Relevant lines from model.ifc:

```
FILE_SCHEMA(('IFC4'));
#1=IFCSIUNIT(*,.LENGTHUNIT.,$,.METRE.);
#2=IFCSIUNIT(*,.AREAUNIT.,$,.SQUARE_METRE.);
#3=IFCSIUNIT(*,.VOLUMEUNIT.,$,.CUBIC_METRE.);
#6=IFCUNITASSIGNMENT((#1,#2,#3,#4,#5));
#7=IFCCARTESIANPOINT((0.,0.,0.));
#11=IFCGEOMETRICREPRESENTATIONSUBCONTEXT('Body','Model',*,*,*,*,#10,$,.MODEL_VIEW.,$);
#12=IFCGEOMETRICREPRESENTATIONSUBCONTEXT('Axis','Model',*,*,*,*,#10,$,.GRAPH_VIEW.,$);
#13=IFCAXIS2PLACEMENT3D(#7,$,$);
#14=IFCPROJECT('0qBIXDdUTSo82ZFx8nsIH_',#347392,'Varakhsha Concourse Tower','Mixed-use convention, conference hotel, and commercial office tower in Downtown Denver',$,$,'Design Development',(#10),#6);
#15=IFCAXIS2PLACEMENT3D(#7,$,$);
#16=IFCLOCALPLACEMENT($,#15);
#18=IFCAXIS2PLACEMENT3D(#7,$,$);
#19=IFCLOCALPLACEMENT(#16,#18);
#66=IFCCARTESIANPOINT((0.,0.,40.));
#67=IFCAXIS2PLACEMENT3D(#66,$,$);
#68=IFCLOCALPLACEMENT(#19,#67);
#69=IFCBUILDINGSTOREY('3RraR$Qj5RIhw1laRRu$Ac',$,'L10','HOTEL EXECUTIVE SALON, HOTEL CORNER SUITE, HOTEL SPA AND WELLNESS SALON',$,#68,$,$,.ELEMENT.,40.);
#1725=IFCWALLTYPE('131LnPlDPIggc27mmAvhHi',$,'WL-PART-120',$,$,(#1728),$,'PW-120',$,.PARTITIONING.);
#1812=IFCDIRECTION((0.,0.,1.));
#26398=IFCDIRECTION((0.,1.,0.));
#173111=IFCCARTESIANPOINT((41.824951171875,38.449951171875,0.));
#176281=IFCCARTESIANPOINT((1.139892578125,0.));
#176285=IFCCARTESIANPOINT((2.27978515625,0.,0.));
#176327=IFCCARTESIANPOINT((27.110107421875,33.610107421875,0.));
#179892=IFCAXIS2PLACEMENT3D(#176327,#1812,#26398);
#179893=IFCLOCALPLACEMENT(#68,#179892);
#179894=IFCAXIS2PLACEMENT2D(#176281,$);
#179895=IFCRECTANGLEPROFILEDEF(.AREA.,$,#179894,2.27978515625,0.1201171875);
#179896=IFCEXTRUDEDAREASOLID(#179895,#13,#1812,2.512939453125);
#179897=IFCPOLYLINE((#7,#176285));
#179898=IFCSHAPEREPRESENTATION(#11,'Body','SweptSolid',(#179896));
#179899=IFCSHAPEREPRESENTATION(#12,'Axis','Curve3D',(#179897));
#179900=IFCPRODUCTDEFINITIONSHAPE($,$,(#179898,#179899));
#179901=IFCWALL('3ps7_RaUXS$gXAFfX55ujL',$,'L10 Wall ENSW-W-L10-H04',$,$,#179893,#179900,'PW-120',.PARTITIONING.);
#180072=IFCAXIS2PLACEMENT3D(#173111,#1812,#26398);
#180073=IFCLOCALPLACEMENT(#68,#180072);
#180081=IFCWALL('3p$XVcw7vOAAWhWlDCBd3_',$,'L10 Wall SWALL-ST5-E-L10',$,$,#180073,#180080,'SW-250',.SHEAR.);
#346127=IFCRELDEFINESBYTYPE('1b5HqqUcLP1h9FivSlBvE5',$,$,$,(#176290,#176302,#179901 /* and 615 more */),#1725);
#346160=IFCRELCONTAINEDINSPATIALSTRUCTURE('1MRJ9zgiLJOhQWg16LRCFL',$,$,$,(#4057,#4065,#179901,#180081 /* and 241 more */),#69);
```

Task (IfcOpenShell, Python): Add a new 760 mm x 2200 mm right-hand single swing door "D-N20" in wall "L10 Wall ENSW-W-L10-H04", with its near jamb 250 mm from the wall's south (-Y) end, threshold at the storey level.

```python
import numpy as np
import ifcopenshell
import ifcopenshell.api.feature
import ifcopenshell.api.geometry
import ifcopenshell.api.root
import ifcopenshell.api.spatial
import ifcopenshell.geom
import ifcopenshell.util.element
import ifcopenshell.util.placement
import ifcopenshell.util.representation
import ifcopenshell.util.shape
import ifcopenshell.util.unit

model = ifcopenshell.open("model.ifc")
unit_scale = ifcopenshell.util.unit.calculate_unit_scale(model)
settings = ifcopenshell.geom.settings()


def volume(element):
    """Net volume in cubic metres, openings subtracted."""
    shape = ifcopenshell.geom.create_shape(settings, element)
    return ifcopenshell.util.shape.get_volume(shape.geometry)


wall = model.by_guid("3ps7_RaUXS$gXAFfX55ujL")
storey = ifcopenshell.util.element.get_container(wall, ifc_class="IfcBuildingStorey")
context = ifcopenshell.util.representation.get_context(model, "Model", "Body", "MODEL_VIEW")
before = volume(wall)

width, height, from_end, sill = 0.76, 2.2, 0.25, 0.0  # metres

# The wall runs along its own X axis, and the end named is its -X end.
wall_shape = ifcopenshell.geom.create_shape(settings, wall)
x, y, z = ifcopenshell.util.shape.get_vertices(wall_shape.geometry).T
start = x.min() + from_end
face, thickness = float(y.min()), float(y.max() - y.min())
wall_matrix = ifcopenshell.util.placement.get_local_placement(wall.ObjectPlacement)
level = ifcopenshell.util.placement.get_local_placement(storey.ObjectPlacement)[2, 3]


def in_wall(x, y):
    """Placement at x, y metres in the wall's axes, at sill height."""
    matrix = wall_matrix.copy()
    matrix[:, 3] = wall_matrix @ np.array([x / unit_scale, y / unit_scale, 0.0, 1.0])
    matrix[2, 3] = level + sill / unit_scale
    return matrix


# Opening: a box that overshoots both wall faces by 50 mm.
opening = ifcopenshell.api.root.create_entity(model, ifc_class="IfcOpeningElement", predefined_type="OPENING")
box = ifcopenshell.api.geometry.add_wall_representation(
    model, context=context, length=width, height=height, thickness=thickness + 0.1
)
ifcopenshell.api.geometry.assign_representation(model, product=opening, representation=box)
ifcopenshell.api.geometry.edit_object_placement(model, product=opening, matrix=in_wall(start, face - 0.05), is_si=False)
ifcopenshell.api.feature.add_feature(model, feature=opening, element=wall)

door = ifcopenshell.api.root.create_entity(model, ifc_class="IfcDoor", name="D-N20", predefined_type="DOOR")
door.OverallWidth, door.OverallHeight = width / unit_scale, height / unit_scale
door.OperationType = "SINGLE_SWING_RIGHT"
body = ifcopenshell.api.geometry.add_door_representation(
    model,
    context=context,
    overall_width=door.OverallWidth,
    overall_height=door.OverallHeight,
    operation_type="SINGLE_SWING_RIGHT",
    lining_properties={"LiningDepth": thickness / unit_scale, "ThresholdDepth": thickness / unit_scale},
)
ifcopenshell.api.geometry.assign_representation(model, product=door, representation=body)
ifcopenshell.api.spatial.assign_container(model, products=[door], relating_structure=storey)
ifcopenshell.api.feature.add_filling(model, opening=opening, element=door)

# The lining spans the wall, so the door starts at the wall face.
ifcopenshell.api.geometry.edit_object_placement(model, product=door, matrix=in_wall(start, face), is_si=False)

after = volume(wall)

print(f"wall volume {before:.3f} -> {after:.3f} m3")

model.write("model_edited.ifc")
```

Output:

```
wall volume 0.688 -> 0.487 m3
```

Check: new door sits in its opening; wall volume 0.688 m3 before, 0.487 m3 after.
